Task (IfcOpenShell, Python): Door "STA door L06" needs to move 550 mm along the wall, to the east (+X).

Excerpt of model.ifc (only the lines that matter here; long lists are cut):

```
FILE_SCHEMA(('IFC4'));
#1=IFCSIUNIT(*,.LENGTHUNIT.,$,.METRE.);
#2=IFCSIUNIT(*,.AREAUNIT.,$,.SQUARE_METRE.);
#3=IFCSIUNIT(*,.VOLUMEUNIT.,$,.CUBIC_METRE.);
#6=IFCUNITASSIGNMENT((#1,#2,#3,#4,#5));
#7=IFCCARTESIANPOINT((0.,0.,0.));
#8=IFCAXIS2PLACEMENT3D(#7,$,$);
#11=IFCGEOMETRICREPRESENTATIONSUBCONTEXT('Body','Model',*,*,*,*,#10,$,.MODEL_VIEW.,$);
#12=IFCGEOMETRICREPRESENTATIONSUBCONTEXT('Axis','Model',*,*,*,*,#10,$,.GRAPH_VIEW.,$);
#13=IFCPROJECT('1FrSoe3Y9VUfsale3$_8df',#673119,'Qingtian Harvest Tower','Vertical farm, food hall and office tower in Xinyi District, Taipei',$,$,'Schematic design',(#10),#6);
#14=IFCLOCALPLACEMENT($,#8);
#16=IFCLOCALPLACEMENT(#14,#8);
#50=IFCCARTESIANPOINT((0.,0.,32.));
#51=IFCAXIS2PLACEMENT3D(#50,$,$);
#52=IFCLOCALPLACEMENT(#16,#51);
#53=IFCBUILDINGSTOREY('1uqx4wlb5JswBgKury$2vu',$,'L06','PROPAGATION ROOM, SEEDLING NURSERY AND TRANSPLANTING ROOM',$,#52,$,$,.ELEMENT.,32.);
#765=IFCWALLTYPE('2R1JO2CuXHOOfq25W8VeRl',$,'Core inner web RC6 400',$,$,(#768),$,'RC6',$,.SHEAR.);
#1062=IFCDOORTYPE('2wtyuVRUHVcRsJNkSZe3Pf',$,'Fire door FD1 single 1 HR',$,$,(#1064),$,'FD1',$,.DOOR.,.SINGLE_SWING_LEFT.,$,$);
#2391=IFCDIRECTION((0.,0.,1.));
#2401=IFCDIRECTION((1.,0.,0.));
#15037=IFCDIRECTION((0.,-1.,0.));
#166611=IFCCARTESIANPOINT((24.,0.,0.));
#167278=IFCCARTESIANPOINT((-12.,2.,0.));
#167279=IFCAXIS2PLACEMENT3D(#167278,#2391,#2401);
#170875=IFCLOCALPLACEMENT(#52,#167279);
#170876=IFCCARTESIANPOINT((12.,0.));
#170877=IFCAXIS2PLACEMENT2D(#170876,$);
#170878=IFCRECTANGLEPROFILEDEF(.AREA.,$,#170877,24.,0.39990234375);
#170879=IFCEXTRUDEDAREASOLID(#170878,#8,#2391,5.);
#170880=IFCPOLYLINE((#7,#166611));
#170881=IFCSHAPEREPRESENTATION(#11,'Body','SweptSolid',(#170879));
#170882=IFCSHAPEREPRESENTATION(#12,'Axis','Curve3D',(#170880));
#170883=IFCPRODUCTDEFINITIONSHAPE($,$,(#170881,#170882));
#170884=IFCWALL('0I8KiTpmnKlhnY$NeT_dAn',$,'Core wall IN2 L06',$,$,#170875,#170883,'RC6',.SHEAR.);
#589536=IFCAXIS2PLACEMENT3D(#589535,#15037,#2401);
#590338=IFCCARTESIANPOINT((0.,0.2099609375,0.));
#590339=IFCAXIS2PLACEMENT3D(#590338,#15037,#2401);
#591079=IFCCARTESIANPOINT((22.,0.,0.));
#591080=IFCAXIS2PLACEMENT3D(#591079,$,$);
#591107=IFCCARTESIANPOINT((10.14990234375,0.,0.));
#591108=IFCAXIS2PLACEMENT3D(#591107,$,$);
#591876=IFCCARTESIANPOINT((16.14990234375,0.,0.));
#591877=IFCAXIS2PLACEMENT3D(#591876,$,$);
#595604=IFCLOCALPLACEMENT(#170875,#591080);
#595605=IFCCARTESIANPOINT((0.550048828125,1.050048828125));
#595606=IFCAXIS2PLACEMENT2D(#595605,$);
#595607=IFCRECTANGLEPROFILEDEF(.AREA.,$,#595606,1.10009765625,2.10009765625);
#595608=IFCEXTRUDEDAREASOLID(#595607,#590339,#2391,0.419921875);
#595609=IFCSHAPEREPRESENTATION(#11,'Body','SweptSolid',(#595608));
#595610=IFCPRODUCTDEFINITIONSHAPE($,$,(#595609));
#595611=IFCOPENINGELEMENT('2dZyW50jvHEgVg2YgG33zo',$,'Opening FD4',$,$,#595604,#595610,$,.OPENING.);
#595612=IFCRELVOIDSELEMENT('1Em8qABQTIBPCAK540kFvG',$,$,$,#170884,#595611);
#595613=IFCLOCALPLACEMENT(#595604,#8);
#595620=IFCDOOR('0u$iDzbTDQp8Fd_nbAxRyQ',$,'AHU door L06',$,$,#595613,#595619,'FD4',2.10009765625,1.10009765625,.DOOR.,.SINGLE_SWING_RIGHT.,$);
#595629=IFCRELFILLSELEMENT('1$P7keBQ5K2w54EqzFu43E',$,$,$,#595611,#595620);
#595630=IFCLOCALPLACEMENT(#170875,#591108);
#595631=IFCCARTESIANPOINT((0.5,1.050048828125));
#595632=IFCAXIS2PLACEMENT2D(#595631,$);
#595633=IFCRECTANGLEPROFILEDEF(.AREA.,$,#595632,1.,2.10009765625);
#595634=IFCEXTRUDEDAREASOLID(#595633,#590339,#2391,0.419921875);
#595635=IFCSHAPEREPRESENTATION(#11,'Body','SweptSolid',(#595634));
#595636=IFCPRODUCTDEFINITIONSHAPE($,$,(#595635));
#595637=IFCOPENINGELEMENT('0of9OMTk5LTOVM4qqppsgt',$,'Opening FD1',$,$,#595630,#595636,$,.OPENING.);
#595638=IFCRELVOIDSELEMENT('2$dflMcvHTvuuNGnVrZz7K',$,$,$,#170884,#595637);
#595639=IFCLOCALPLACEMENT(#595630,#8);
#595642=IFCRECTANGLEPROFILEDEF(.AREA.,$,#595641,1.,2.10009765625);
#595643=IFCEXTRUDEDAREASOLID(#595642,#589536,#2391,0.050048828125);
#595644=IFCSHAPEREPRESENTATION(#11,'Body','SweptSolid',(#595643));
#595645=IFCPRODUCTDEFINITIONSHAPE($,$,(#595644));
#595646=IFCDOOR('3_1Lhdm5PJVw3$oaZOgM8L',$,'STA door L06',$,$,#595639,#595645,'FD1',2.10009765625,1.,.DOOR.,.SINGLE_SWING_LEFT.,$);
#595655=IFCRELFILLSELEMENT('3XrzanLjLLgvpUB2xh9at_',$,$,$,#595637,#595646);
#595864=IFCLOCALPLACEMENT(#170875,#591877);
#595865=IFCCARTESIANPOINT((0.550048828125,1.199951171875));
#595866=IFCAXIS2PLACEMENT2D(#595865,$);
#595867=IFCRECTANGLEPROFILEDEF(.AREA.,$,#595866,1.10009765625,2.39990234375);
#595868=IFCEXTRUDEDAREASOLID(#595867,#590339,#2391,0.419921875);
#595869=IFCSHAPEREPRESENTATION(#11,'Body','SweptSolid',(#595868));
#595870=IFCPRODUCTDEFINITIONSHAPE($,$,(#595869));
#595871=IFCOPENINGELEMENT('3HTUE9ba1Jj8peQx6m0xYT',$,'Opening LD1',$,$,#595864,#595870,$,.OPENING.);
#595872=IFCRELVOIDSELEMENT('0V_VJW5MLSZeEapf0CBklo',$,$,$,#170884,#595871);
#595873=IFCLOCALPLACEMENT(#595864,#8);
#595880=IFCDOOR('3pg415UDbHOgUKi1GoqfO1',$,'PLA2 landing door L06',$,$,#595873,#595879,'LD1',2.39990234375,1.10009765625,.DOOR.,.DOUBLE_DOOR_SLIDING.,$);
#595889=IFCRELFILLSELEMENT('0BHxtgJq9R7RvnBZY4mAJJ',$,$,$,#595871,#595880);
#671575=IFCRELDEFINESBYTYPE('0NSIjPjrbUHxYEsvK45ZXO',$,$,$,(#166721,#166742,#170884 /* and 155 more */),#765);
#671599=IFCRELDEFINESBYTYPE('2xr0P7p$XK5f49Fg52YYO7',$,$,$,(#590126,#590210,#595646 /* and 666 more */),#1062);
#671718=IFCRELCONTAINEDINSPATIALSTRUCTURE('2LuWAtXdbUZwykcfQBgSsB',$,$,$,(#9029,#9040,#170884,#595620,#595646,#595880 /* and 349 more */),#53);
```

```python
import ifcopenshell
import ifcopenshell.api.geometry
import ifcopenshell.util.placement

model = ifcopenshell.open("model.ifc")

door = model.by_guid("3_1Lhdm5PJVw3$oaZOgM8L")
opening = door.FillsVoids[0].RelatingOpeningElement
wall = opening.VoidsElements[0].RelatingBuildingElement

wall_matrix = ifcopenshell.util.placement.get_local_placement(wall.ObjectPlacement)
shift = wall_matrix[:3, 0] * 0.55
before = ifcopenshell.util.placement.get_local_placement(door.ObjectPlacement)[:3, 3].copy()

# The door is placed relative to its opening, so it follows when the opening moves.
matrix = ifcopenshell.util.placement.get_local_placement(opening.ObjectPlacement)
matrix[:3, 3] += shift
ifcopenshell.api.geometry.edit_object_placement(
    model, product=opening, matrix=matrix, is_si=False, should_transform_children=True
)

after = ifcopenshell.util.placement.get_local_placement(door.ObjectPlacement)[:3, 3]
print("door moved by", (after - before).round(3) + 0.0)

model.write("model_v2.ifc")
```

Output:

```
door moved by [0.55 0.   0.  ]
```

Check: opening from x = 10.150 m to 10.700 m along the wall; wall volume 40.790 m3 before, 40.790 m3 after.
